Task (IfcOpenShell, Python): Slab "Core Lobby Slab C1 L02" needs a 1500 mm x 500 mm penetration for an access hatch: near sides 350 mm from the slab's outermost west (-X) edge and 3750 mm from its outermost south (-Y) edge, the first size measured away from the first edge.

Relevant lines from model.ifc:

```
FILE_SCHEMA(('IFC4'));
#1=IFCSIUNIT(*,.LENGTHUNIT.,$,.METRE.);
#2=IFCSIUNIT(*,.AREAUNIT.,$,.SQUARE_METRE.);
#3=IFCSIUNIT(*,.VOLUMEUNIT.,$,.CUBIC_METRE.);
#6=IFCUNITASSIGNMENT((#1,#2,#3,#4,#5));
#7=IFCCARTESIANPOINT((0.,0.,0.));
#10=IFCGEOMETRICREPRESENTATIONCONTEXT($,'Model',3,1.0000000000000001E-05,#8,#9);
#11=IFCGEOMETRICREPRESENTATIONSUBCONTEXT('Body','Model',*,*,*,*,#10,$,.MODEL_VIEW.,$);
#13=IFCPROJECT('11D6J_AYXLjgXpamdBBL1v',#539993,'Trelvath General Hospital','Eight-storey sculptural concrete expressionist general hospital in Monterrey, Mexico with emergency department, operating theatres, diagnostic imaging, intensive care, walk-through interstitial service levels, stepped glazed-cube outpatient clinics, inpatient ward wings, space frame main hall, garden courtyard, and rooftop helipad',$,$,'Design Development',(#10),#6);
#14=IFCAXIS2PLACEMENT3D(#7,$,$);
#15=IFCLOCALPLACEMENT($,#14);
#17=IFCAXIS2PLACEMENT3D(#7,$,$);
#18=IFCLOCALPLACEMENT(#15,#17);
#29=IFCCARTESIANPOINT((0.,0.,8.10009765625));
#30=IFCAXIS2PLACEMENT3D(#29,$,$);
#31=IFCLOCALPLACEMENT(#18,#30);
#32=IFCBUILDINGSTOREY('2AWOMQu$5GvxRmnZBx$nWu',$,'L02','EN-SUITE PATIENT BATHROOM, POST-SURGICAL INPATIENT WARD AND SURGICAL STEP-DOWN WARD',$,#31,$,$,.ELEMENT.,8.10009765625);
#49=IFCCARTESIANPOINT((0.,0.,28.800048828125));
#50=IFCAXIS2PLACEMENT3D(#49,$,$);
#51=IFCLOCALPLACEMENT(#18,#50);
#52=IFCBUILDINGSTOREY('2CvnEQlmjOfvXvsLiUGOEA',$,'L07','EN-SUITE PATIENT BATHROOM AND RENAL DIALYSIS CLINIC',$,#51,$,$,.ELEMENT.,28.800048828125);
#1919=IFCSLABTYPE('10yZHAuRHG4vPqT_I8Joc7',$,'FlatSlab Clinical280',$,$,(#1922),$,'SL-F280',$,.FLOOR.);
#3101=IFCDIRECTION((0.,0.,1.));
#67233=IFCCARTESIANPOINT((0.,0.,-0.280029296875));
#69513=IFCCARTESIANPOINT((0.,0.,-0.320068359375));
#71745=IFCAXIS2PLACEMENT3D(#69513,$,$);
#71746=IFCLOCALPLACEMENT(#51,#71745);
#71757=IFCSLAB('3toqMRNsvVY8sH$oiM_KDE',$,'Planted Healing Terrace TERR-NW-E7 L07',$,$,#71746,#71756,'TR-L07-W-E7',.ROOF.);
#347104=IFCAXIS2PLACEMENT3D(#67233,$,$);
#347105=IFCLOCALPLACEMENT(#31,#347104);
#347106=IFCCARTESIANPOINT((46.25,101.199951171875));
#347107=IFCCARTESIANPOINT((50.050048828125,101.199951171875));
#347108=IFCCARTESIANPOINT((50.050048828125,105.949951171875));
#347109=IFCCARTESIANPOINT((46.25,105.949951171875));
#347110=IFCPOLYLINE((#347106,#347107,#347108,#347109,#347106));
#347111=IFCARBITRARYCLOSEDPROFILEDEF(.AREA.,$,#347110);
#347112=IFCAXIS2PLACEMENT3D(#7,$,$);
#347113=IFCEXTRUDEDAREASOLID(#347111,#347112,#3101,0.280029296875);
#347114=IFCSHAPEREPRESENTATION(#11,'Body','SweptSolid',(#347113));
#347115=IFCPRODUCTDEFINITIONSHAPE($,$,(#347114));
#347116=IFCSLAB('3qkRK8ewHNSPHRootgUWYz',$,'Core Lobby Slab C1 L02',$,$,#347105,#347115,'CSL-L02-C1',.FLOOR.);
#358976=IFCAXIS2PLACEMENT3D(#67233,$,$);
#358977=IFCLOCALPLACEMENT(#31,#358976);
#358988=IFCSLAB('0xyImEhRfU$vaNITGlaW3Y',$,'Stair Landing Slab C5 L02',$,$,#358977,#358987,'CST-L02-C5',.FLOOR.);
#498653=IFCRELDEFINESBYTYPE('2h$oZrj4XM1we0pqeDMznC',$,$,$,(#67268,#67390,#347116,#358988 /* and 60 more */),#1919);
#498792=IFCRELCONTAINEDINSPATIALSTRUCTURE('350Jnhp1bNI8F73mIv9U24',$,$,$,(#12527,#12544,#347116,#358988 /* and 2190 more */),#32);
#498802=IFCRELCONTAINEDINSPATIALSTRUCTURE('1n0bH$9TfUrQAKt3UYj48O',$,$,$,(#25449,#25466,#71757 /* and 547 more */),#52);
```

```python
import numpy as np
import ifcopenshell
import ifcopenshell.api.feature
import ifcopenshell.api.geometry
import ifcopenshell.api.root
import ifcopenshell.geom
import ifcopenshell.util.placement
import ifcopenshell.util.representation
import ifcopenshell.util.shape
import ifcopenshell.util.unit

model = ifcopenshell.open("model.ifc")
unit_scale = ifcopenshell.util.unit.calculate_unit_scale(model)
settings = ifcopenshell.geom.settings()


def volume(element):
    """Net volume in cubic metres, openings subtracted."""
    shape = ifcopenshell.geom.create_shape(settings, element)
    return ifcopenshell.util.shape.get_volume(shape.geometry)


slab = model.by_guid("3qkRK8ewHNSPHRootgUWYz")
before = volume(slab)

# Extent in the slab's own axes, in metres. The edges named are its -X and -Y sides.
slab_shape = ifcopenshell.geom.create_shape(settings, slab)
vertices = ifcopenshell.util.shape.get_vertices(slab_shape.geometry)
x_min, y_min, bottom = vertices.min(axis=0)
top = vertices[:, 2].max()

opening = ifcopenshell.api.root.create_entity(model, ifc_class="IfcOpeningElement", name="Access hatch opening", predefined_type="OPENING")
context = ifcopenshell.util.representation.get_context(model, "Model", "Body", "MODEL_VIEW")
width, depth = 1.5, 0.5
outline = [(0.0, 0.0), (width, 0.0), (width, depth), (0.0, depth), (0.0, 0.0)]
# Overshoot both faces by 50 mm so the cut is clean.
shape = ifcopenshell.api.geometry.add_slab_representation(
    model, context=context, depth=top - bottom + 0.1, polyline=outline
)
ifcopenshell.api.geometry.assign_representation(model, product=opening, representation=shape)

matrix = ifcopenshell.util.placement.get_local_placement(slab.ObjectPlacement)
matrix[:, 3] = matrix @ np.append(np.array([x_min + 0.35, y_min + 3.75, bottom - 0.05]) / unit_scale, 1.0)
ifcopenshell.api.geometry.edit_object_placement(model, product=opening, matrix=matrix, is_si=False)
ifcopenshell.api.feature.add_feature(model, feature=opening, element=slab)

after = volume(slab)

print(f"slab volume {before:.3f} -> {after:.3f} m3")

model.write("model-out.ifc")
```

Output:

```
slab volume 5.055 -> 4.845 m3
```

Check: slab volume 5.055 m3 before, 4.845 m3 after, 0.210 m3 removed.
